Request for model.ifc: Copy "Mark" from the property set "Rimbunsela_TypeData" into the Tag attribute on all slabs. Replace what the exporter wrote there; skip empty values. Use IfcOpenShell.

First a look at what the model holds.

```python
import ifcopenshell
import ifcopenshell.util.element

model = ifcopenshell.open("model.ifc")
print(model.schema)
slabs = model.by_type("IfcSlab")
print(len(slabs), "slabs")
for e in slabs[:8]:
    source = ifcopenshell.util.element.get_pset(e, "Rimbunsela_TypeData", "Mark")
    target = e.Tag
    print(e.id(), repr(source), repr(target), sep=" | ")
```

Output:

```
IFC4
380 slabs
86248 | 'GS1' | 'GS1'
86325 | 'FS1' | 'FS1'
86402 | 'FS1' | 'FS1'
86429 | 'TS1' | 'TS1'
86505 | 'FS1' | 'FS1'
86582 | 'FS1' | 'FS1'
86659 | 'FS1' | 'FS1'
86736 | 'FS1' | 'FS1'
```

```python
import ifcopenshell
import ifcopenshell.util.element

model = ifcopenshell.open("model.ifc")

count = 0
for e in model.by_type("IfcSlab"):
    value = ifcopenshell.util.element.get_pset(e, "Rimbunsela_TypeData", "Mark")
    current = e.Tag
    if not value or not value.strip() or current == value:
        continue
    e.Tag = value
    count += 1

print(count, "slabs updated")

model.write("model_rev.ifc")
```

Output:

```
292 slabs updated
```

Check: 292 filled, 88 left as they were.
